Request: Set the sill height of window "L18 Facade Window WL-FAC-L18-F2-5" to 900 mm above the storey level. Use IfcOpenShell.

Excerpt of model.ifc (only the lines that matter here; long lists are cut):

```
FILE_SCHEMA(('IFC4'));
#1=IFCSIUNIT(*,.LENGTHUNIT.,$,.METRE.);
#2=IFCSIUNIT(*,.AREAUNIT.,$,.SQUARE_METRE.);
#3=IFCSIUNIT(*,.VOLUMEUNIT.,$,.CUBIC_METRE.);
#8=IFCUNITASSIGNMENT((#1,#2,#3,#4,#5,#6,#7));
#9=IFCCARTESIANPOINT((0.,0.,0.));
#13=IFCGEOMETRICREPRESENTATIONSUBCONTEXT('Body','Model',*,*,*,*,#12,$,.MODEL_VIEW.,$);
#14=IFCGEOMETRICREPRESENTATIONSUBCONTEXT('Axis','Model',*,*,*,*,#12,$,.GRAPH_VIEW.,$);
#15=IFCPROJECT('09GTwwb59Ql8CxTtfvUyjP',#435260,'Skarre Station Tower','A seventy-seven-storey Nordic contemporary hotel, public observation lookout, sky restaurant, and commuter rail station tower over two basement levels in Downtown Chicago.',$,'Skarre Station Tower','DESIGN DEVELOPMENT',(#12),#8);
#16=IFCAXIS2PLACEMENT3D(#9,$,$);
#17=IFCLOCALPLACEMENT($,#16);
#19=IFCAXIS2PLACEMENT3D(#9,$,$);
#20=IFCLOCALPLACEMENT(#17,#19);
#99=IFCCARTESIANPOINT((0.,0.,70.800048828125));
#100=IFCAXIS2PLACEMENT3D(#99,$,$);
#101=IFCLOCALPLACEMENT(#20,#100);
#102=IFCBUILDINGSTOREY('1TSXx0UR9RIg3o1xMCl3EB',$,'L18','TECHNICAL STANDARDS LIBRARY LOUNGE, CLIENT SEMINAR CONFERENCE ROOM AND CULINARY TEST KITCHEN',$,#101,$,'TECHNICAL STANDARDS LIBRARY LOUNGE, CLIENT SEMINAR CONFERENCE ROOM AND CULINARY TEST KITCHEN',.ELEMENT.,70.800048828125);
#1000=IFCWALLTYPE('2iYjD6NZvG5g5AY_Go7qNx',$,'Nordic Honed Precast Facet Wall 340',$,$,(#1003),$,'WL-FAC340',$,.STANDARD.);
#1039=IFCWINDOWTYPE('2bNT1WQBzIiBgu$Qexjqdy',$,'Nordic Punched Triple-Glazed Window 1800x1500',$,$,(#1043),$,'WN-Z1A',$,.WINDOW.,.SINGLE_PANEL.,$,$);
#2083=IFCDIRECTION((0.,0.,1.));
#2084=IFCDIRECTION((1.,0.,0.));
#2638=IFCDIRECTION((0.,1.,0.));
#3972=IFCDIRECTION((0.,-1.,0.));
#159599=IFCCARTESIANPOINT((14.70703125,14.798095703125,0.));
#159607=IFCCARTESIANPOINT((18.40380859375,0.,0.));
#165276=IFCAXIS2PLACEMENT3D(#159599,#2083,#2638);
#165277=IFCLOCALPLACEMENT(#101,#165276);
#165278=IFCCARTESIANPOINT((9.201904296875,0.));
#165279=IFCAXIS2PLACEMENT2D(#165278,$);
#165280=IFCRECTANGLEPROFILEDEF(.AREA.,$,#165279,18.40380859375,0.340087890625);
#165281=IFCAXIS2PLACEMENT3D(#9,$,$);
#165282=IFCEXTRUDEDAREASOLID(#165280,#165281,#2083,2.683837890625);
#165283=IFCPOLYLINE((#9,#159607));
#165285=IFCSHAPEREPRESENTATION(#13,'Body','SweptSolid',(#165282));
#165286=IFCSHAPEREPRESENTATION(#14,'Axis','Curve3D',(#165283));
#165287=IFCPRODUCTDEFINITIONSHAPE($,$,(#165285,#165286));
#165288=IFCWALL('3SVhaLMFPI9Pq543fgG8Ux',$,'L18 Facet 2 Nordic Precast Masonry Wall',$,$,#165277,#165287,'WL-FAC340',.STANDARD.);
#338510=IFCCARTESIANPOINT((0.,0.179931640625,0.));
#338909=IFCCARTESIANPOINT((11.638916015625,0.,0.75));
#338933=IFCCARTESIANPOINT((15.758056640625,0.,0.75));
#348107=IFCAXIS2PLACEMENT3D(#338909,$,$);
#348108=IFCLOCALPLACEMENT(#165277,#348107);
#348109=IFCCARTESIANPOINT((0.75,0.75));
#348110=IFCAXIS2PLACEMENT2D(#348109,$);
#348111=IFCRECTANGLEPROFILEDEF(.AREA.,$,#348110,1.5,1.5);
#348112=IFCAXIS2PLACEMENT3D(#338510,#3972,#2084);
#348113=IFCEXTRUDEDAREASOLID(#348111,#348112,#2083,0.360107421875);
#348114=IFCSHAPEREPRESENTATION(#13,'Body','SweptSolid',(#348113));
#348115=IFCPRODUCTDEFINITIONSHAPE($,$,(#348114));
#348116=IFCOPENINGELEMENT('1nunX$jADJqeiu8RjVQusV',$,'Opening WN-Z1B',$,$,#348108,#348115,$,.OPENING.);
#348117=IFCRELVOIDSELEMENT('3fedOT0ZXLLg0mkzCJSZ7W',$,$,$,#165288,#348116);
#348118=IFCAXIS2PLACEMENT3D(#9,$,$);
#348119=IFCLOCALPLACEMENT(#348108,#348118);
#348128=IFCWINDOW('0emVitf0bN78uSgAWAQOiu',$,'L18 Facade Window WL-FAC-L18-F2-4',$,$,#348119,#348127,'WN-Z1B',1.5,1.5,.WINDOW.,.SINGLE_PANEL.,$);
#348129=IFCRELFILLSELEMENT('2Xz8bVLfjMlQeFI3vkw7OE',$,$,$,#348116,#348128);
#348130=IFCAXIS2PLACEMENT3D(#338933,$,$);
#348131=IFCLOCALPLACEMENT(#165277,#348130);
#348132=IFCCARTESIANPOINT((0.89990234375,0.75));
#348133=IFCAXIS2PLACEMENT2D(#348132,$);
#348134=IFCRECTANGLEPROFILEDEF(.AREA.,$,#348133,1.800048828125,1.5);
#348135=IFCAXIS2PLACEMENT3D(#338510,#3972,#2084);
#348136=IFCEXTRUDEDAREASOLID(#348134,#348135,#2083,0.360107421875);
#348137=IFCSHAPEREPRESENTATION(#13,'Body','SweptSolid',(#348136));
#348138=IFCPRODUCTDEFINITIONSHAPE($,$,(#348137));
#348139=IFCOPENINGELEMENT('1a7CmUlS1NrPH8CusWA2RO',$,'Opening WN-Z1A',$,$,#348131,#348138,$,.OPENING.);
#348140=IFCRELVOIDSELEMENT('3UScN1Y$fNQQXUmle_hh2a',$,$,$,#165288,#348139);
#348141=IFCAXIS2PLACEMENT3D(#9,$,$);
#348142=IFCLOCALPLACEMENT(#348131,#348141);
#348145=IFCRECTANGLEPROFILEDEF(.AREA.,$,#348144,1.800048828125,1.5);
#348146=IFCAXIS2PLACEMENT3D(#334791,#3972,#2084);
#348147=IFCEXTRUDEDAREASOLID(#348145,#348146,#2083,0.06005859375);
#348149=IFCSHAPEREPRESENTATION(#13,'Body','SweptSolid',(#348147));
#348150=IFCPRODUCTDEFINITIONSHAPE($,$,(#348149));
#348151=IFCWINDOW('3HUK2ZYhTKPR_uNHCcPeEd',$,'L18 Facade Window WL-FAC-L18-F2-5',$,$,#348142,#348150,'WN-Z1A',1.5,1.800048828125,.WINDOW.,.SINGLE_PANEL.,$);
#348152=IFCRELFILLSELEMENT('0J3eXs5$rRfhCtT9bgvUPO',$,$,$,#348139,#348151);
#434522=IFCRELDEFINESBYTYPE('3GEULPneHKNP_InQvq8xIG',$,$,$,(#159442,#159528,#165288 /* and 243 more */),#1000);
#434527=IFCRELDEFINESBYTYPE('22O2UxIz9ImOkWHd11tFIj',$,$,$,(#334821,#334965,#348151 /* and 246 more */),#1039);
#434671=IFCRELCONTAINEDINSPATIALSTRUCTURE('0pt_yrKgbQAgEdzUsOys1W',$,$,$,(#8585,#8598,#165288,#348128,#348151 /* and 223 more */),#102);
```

```python
import numpy as np
import ifcopenshell
import ifcopenshell.api.geometry
import ifcopenshell.geom
import ifcopenshell.util.element
import ifcopenshell.util.placement
import ifcopenshell.util.shape
import ifcopenshell.util.unit

model = ifcopenshell.open("model.ifc")
unit_scale = ifcopenshell.util.unit.calculate_unit_scale(model)

window = model.by_id(348151)
opening = window.FillsVoids[0].RelatingOpeningElement
storey = ifcopenshell.util.element.get_container(window, ifc_class="IfcBuildingStorey")
level = ifcopenshell.util.placement.get_local_placement(storey.ObjectPlacement)[2, 3]

# The opening's origin need not be at the sill, so measure its lowest point.
shape = ifcopenshell.geom.create_shape(ifcopenshell.geom.settings(), opening)
bottom = ifcopenshell.util.shape.get_shape_bottom_elevation(shape, shape.geometry) / unit_scale
dz = level + 0.9 / unit_scale - bottom

shift = np.array([0.0, 0.0, dz])
# The window is placed relative to its opening, so it follows when the opening moves.
matrix = ifcopenshell.util.placement.get_local_placement(opening.ObjectPlacement)
matrix[:3, 3] += shift
ifcopenshell.api.geometry.edit_object_placement(
    model, product=opening, matrix=matrix, is_si=False, should_transform_children=True
)

print(f"moved by {dz * unit_scale:+.3f} m")

model.write("model_edited.ifc")
```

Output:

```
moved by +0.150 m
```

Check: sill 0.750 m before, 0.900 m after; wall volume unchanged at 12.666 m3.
